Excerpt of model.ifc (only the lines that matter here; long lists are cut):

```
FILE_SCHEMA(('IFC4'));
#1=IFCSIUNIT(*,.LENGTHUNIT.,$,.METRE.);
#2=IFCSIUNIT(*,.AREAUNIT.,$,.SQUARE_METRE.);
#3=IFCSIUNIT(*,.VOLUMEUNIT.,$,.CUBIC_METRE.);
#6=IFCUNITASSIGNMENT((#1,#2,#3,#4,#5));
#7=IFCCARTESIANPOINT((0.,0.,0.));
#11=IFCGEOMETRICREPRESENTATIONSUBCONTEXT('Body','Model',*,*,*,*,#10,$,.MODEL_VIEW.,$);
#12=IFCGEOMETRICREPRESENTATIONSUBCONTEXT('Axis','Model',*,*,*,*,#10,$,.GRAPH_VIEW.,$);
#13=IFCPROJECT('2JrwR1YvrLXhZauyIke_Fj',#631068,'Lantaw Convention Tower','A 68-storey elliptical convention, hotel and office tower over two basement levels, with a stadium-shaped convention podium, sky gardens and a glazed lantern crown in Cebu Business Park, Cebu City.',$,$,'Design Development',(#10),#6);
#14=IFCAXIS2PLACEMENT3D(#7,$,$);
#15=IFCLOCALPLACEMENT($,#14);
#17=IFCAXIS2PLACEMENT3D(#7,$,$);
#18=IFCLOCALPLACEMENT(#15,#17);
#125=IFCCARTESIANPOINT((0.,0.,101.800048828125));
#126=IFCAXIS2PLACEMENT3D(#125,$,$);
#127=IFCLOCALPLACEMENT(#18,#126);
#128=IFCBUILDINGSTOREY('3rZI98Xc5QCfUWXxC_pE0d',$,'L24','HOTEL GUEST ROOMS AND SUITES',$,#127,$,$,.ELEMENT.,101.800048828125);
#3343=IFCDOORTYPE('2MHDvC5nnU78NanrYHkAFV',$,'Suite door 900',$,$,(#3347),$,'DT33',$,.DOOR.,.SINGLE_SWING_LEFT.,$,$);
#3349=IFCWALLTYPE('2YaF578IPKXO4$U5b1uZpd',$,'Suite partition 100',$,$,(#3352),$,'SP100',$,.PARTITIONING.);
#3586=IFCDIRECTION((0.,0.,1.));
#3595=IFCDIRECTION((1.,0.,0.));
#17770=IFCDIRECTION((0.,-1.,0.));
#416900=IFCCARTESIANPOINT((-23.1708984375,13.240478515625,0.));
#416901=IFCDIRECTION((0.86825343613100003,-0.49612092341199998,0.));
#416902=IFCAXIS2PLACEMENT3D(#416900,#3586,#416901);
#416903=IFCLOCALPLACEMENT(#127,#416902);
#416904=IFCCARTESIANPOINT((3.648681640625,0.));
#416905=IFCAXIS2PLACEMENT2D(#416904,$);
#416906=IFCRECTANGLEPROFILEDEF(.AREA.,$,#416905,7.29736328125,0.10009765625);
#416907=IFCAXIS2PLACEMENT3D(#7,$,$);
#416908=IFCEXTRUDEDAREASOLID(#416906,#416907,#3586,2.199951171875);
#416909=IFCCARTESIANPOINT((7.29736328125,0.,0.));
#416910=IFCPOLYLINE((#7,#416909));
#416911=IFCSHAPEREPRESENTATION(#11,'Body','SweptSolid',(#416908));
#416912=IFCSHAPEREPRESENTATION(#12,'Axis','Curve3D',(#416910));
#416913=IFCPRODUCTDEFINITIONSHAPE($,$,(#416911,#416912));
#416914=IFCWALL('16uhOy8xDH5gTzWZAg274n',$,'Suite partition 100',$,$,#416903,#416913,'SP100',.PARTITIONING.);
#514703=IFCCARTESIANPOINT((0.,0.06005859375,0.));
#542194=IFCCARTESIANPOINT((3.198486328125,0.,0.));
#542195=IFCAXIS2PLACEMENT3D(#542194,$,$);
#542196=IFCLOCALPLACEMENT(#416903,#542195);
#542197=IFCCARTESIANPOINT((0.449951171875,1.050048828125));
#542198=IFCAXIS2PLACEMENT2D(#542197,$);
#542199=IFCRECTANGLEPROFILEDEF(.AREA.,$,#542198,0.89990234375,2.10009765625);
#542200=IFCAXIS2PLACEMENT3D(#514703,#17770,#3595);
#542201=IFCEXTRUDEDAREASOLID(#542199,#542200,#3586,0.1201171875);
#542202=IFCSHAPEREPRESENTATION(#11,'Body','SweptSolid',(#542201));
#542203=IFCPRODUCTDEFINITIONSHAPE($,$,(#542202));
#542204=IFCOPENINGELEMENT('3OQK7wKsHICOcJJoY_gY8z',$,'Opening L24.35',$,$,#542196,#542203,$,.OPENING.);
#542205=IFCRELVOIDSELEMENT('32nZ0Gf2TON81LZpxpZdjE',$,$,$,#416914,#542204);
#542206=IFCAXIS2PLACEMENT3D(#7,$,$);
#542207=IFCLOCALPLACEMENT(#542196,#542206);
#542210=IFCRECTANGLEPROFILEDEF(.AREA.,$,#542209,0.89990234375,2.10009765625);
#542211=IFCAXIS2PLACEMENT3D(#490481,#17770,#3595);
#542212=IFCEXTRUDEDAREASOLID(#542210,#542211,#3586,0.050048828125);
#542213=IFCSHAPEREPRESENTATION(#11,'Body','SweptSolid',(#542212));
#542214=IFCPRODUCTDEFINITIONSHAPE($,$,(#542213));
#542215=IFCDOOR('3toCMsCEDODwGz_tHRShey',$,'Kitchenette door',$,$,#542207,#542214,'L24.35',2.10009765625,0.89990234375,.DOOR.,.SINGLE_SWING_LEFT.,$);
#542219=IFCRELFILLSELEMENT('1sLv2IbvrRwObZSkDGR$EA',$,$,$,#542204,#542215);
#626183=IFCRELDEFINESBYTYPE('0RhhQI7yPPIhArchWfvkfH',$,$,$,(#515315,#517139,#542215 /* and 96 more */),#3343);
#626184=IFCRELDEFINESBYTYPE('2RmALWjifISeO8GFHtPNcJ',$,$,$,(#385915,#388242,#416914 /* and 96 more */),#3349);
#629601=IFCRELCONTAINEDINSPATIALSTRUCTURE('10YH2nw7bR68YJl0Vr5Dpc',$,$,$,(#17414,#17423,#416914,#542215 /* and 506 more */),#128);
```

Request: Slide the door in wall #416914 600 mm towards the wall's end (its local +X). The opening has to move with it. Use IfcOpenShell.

```python
import ifcopenshell
import ifcopenshell.api.geometry
import ifcopenshell.util.placement

model = ifcopenshell.open("model.ifc")

door = model.by_guid("3toCMsCEDODwGz_tHRShey")
opening = door.FillsVoids[0].RelatingOpeningElement
wall = opening.VoidsElements[0].RelatingBuildingElement

wall_matrix = ifcopenshell.util.placement.get_local_placement(wall.ObjectPlacement)
shift = wall_matrix[:3, 0] * 0.6
before = ifcopenshell.util.placement.get_local_placement(door.ObjectPlacement)[:3, 3].copy()

# The door is placed relative to its opening, so it follows when the opening moves.
matrix = ifcopenshell.util.placement.get_local_placement(opening.ObjectPlacement)
matrix[:3, 3] += shift
ifcopenshell.api.geometry.edit_object_placement(
    model, product=opening, matrix=matrix, is_si=False, should_transform_children=True
)

after = ifcopenshell.util.placement.get_local_placement(door.ObjectPlacement)[:3, 3]
print("door moved by", (after - before).round(3) + 0.0)

model.write("model_edited.ifc")
```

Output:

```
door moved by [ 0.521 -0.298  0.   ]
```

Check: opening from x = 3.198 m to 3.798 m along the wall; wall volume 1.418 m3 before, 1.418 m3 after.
